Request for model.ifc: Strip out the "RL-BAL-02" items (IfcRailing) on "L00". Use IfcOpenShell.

First a look at what the model holds.

```python
import ifcopenshell
import ifcopenshell.util.element

model = ifcopenshell.open("model.ifc")
print(model.schema)
storey = next(s for s in model.by_type("IfcBuildingStorey") if s.Name == "L00")
railings = [e for e in ifcopenshell.util.element.get_decomposition(storey) if e.is_a("IfcRailing")]
seen = {}
for e in railings:
    element_type = ifcopenshell.util.element.get_type(e)
    name = element_type.Name if element_type not in (None, e) else None
    seen[name] = seen.get(name, 0) + 1
for name, count in sorted(seen.items(), key=str):
    print(count, "x", name)
```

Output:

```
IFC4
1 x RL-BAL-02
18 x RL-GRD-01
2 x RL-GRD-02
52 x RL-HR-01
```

```python
import ifcopenshell
import ifcopenshell.api.root
import ifcopenshell.util.element

model = ifcopenshell.open("model.ifc")

storey = next(s for s in model.by_type("IfcBuildingStorey") if s.Name == "L00")
railings = [e for e in ifcopenshell.util.element.get_decomposition(storey) if e.is_a("IfcRailing")]
targets = [e for e in railings if (t := ifcopenshell.util.element.get_type(e)) not in (None, e) and t.Name == "RL-BAL-02"]

for e in targets:
    ifcopenshell.api.root.remove_product(model, product=e)
print(len(targets), "removed")

model.write("model_rev.ifc")
```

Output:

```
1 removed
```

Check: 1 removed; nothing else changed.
